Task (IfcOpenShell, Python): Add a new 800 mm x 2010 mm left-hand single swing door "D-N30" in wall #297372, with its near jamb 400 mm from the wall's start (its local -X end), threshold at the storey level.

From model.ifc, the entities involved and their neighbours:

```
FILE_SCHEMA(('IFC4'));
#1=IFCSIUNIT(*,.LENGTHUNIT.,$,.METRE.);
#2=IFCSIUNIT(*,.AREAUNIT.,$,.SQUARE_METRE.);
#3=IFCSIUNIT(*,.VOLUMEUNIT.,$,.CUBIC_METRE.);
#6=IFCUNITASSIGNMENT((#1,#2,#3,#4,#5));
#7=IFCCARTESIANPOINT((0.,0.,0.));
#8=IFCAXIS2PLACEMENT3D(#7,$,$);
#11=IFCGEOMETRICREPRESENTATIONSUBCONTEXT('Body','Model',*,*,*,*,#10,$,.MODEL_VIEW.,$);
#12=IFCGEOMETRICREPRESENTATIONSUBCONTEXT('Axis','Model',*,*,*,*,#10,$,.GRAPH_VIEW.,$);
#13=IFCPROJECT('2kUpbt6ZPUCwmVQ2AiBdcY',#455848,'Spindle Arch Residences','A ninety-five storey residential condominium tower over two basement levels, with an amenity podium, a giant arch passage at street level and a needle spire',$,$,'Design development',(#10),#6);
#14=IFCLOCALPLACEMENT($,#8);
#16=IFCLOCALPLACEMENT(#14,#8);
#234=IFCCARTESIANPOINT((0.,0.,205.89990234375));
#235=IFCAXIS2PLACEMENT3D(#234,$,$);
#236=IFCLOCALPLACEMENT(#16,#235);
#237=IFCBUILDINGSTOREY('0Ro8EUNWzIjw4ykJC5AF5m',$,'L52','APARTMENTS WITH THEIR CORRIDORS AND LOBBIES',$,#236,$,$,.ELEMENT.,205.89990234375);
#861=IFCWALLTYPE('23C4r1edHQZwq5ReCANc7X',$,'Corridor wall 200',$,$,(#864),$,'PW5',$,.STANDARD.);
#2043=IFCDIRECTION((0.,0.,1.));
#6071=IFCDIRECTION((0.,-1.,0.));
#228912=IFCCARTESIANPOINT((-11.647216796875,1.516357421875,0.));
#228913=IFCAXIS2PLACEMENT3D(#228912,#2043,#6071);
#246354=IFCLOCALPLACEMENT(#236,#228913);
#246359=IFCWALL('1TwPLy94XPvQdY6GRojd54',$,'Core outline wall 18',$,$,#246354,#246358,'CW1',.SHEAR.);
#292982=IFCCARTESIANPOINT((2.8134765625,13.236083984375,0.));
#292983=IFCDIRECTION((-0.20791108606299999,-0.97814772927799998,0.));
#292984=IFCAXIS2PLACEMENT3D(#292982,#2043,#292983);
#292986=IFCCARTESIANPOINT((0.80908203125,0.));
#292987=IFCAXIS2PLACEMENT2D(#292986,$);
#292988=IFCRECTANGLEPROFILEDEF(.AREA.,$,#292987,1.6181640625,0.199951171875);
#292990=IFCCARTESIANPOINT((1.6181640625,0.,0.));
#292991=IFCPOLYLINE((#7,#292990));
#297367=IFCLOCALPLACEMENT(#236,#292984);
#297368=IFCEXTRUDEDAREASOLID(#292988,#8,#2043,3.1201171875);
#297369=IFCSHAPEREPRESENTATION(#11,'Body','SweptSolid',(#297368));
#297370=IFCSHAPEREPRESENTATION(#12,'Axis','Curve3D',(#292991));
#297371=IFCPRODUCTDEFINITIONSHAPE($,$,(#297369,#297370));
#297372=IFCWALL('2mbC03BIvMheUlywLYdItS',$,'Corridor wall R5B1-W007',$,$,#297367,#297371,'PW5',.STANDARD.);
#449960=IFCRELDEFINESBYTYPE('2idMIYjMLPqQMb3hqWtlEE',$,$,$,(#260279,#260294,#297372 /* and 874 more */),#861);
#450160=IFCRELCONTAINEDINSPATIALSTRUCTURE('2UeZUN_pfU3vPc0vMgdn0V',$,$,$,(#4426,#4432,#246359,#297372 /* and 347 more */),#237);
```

```python
import numpy as np
import ifcopenshell
import ifcopenshell.api.feature
import ifcopenshell.api.geometry
import ifcopenshell.api.root
import ifcopenshell.api.spatial
import ifcopenshell.geom
import ifcopenshell.util.element
import ifcopenshell.util.placement
import ifcopenshell.util.representation
import ifcopenshell.util.shape
import ifcopenshell.util.unit

model = ifcopenshell.open("model.ifc")
unit_scale = ifcopenshell.util.unit.calculate_unit_scale(model)
settings = ifcopenshell.geom.settings()


def volume(element):
    """Net volume in cubic metres, openings subtracted."""
    shape = ifcopenshell.geom.create_shape(settings, element)
    return ifcopenshell.util.shape.get_volume(shape.geometry)


wall = model.by_guid("2mbC03BIvMheUlywLYdItS")
storey = ifcopenshell.util.element.get_container(wall, ifc_class="IfcBuildingStorey")
context = ifcopenshell.util.representation.get_context(model, "Model", "Body", "MODEL_VIEW")
before = volume(wall)

width, height, from_end, sill = 0.8, 2.01, 0.4, 0.0  # metres

# The wall runs along its own X axis, and the end named is its -X end.
wall_shape = ifcopenshell.geom.create_shape(settings, wall)
x, y, z = ifcopenshell.util.shape.get_vertices(wall_shape.geometry).T
start = x.min() + from_end
face, thickness = float(y.min()), float(y.max() - y.min())
wall_matrix = ifcopenshell.util.placement.get_local_placement(wall.ObjectPlacement)
level = ifcopenshell.util.placement.get_local_placement(storey.ObjectPlacement)[2, 3]


def in_wall(x, y):
    """Placement at x, y metres in the wall's axes, at sill height."""
    matrix = wall_matrix.copy()
    matrix[:, 3] = wall_matrix @ np.array([x / unit_scale, y / unit_scale, 0.0, 1.0])
    matrix[2, 3] = level + sill / unit_scale
    return matrix


# Opening: a box that overshoots both wall faces by 50 mm.
opening = ifcopenshell.api.root.create_entity(model, ifc_class="IfcOpeningElement", predefined_type="OPENING")
box = ifcopenshell.api.geometry.add_wall_representation(
    model, context=context, length=width, height=height, thickness=thickness + 0.1
)
ifcopenshell.api.geometry.assign_representation(model, product=opening, representation=box)
ifcopenshell.api.geometry.edit_object_placement(model, product=opening, matrix=in_wall(start, face - 0.05), is_si=False)
ifcopenshell.api.feature.add_feature(model, feature=opening, element=wall)

door = ifcopenshell.api.root.create_entity(model, ifc_class="IfcDoor", name="D-N30", predefined_type="DOOR")
door.OverallWidth, door.OverallHeight = width / unit_scale, height / unit_scale
door.OperationType = "SINGLE_SWING_LEFT"
body = ifcopenshell.api.geometry.add_door_representation(
    model,
    context=context,
    overall_width=door.OverallWidth,
    overall_height=door.OverallHeight,
    operation_type="SINGLE_SWING_LEFT",
    lining_properties={"LiningDepth": thickness / unit_scale, "ThresholdDepth": thickness / unit_scale},
)
ifcopenshell.api.geometry.assign_representation(model, product=door, representation=body)
ifcopenshell.api.spatial.assign_container(model, products=[door], relating_structure=storey)
ifcopenshell.api.feature.add_filling(model, opening=opening, element=door)

# The lining spans the wall, so the door starts at the wall face.
ifcopenshell.api.geometry.edit_object_placement(model, product=door, matrix=in_wall(start, face), is_si=False)

after = volume(wall)

print(f"wall volume {before:.3f} -> {after:.3f} m3")

model.write("model_v2.ifc")
```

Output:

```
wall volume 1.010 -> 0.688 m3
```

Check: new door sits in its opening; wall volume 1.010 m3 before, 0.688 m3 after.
